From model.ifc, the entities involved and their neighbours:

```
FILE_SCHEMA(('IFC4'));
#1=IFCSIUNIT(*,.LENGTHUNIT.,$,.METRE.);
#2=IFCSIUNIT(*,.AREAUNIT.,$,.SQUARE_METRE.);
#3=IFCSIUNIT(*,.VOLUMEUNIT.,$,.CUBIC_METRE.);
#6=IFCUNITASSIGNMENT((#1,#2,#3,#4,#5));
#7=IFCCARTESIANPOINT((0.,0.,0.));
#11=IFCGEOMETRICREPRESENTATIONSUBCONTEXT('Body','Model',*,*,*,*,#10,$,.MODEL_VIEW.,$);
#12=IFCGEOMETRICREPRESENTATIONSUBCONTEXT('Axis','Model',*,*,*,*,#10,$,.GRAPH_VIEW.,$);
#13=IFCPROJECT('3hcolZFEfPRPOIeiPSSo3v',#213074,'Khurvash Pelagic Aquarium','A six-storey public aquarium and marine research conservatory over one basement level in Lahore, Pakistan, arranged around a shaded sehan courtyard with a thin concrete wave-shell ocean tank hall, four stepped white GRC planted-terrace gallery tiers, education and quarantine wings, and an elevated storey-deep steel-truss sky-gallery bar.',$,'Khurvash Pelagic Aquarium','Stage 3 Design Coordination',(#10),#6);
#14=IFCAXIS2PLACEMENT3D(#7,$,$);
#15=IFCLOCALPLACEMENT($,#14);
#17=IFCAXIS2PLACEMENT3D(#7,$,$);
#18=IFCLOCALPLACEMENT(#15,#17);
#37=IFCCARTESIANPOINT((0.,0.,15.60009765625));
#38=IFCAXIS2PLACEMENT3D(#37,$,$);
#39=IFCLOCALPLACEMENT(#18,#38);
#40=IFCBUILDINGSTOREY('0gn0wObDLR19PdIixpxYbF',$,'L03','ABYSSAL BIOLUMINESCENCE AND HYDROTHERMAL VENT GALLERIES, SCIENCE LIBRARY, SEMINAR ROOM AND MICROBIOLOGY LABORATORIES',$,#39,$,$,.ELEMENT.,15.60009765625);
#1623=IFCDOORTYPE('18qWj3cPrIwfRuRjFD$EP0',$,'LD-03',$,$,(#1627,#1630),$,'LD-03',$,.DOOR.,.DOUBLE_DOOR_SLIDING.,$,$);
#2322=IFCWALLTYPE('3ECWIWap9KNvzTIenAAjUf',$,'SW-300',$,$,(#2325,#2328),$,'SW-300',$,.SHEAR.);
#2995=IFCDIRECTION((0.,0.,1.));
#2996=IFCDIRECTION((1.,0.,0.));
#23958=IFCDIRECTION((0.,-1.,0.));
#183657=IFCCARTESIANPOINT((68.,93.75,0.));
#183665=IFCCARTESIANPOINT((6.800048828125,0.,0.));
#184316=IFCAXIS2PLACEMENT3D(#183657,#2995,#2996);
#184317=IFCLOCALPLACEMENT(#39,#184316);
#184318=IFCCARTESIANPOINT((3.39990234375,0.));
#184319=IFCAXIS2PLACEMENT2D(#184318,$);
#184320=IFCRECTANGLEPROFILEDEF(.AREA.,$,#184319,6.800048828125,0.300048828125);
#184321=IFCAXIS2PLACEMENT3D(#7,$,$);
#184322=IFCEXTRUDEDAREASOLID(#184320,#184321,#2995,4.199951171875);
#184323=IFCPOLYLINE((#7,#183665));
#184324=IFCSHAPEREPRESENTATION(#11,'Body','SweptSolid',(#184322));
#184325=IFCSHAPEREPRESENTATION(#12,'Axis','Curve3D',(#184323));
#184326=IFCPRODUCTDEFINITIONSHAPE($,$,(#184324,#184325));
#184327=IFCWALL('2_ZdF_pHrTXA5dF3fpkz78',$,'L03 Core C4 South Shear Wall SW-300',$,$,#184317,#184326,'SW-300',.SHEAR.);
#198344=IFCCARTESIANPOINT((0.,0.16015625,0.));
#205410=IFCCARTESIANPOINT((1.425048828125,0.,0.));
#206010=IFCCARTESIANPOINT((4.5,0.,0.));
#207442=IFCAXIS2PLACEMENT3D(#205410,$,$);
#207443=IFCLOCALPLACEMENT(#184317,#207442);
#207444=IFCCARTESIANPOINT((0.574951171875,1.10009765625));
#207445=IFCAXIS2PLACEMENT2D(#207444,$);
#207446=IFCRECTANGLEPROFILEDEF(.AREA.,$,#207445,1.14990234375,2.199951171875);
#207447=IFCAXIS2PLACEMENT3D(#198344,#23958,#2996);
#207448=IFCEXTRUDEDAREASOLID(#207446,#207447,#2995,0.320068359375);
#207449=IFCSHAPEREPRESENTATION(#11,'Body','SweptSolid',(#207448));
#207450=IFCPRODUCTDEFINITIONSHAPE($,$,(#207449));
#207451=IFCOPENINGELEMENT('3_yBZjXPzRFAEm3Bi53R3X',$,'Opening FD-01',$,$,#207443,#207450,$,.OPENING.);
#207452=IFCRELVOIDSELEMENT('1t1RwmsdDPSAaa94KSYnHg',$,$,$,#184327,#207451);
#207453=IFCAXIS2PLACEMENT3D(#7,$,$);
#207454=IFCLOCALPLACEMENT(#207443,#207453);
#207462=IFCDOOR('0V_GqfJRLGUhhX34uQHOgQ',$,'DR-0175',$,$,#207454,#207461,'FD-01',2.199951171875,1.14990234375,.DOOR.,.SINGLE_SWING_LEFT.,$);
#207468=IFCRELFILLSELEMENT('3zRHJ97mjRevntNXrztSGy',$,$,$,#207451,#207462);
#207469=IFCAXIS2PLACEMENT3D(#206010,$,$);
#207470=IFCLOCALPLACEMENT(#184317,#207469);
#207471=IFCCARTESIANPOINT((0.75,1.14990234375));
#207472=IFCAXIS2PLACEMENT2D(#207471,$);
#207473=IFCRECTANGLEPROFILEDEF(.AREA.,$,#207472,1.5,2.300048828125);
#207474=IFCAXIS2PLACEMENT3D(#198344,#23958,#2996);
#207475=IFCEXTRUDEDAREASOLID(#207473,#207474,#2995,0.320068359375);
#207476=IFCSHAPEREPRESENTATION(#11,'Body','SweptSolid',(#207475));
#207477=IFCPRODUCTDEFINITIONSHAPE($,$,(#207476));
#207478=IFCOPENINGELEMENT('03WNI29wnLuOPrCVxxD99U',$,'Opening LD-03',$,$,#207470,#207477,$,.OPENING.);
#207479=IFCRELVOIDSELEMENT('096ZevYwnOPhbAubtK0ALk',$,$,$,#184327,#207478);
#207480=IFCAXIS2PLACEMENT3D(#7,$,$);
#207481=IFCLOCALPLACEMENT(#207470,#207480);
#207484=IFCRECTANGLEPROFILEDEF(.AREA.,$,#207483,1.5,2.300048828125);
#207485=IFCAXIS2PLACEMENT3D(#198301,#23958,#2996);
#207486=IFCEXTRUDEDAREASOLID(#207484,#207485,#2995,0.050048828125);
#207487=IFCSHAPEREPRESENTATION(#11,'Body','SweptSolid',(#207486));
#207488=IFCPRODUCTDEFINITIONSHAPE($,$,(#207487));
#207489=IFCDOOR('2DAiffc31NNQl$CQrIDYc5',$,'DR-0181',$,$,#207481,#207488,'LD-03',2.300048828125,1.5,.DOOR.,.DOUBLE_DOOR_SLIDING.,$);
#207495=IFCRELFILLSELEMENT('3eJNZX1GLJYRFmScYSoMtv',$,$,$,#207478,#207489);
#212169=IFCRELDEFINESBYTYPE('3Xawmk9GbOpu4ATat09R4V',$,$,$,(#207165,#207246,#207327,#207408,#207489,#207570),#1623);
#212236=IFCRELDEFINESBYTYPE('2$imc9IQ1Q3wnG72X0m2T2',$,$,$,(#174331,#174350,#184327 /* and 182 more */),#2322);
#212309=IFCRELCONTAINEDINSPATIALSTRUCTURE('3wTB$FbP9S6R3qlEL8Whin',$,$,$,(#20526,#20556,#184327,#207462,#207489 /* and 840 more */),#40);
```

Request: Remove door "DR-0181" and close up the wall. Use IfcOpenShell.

```python
import ifcopenshell
import ifcopenshell.api.feature
import ifcopenshell.api.root
import ifcopenshell.geom
import ifcopenshell.util.shape

model = ifcopenshell.open("model.ifc")
settings = ifcopenshell.geom.settings()


def volume(element):
    """Net volume in cubic metres, openings subtracted."""
    shape = ifcopenshell.geom.create_shape(settings, element)
    return ifcopenshell.util.shape.get_volume(shape.geometry)


door = model.by_id(207489)
opening = door.FillsVoids[0].RelatingOpeningElement
wall = opening.VoidsElements[0].RelatingBuildingElement
before = volume(wall)

ifcopenshell.api.root.remove_product(model, product=door)
ifcopenshell.api.feature.remove_feature(model, feature=opening)

after = volume(wall)

print(f"wall volume {before:.3f} -> {after:.3f} m3")

model.write("model-out.ifc")
```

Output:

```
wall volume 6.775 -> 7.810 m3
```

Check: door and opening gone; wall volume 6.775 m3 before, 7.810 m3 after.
